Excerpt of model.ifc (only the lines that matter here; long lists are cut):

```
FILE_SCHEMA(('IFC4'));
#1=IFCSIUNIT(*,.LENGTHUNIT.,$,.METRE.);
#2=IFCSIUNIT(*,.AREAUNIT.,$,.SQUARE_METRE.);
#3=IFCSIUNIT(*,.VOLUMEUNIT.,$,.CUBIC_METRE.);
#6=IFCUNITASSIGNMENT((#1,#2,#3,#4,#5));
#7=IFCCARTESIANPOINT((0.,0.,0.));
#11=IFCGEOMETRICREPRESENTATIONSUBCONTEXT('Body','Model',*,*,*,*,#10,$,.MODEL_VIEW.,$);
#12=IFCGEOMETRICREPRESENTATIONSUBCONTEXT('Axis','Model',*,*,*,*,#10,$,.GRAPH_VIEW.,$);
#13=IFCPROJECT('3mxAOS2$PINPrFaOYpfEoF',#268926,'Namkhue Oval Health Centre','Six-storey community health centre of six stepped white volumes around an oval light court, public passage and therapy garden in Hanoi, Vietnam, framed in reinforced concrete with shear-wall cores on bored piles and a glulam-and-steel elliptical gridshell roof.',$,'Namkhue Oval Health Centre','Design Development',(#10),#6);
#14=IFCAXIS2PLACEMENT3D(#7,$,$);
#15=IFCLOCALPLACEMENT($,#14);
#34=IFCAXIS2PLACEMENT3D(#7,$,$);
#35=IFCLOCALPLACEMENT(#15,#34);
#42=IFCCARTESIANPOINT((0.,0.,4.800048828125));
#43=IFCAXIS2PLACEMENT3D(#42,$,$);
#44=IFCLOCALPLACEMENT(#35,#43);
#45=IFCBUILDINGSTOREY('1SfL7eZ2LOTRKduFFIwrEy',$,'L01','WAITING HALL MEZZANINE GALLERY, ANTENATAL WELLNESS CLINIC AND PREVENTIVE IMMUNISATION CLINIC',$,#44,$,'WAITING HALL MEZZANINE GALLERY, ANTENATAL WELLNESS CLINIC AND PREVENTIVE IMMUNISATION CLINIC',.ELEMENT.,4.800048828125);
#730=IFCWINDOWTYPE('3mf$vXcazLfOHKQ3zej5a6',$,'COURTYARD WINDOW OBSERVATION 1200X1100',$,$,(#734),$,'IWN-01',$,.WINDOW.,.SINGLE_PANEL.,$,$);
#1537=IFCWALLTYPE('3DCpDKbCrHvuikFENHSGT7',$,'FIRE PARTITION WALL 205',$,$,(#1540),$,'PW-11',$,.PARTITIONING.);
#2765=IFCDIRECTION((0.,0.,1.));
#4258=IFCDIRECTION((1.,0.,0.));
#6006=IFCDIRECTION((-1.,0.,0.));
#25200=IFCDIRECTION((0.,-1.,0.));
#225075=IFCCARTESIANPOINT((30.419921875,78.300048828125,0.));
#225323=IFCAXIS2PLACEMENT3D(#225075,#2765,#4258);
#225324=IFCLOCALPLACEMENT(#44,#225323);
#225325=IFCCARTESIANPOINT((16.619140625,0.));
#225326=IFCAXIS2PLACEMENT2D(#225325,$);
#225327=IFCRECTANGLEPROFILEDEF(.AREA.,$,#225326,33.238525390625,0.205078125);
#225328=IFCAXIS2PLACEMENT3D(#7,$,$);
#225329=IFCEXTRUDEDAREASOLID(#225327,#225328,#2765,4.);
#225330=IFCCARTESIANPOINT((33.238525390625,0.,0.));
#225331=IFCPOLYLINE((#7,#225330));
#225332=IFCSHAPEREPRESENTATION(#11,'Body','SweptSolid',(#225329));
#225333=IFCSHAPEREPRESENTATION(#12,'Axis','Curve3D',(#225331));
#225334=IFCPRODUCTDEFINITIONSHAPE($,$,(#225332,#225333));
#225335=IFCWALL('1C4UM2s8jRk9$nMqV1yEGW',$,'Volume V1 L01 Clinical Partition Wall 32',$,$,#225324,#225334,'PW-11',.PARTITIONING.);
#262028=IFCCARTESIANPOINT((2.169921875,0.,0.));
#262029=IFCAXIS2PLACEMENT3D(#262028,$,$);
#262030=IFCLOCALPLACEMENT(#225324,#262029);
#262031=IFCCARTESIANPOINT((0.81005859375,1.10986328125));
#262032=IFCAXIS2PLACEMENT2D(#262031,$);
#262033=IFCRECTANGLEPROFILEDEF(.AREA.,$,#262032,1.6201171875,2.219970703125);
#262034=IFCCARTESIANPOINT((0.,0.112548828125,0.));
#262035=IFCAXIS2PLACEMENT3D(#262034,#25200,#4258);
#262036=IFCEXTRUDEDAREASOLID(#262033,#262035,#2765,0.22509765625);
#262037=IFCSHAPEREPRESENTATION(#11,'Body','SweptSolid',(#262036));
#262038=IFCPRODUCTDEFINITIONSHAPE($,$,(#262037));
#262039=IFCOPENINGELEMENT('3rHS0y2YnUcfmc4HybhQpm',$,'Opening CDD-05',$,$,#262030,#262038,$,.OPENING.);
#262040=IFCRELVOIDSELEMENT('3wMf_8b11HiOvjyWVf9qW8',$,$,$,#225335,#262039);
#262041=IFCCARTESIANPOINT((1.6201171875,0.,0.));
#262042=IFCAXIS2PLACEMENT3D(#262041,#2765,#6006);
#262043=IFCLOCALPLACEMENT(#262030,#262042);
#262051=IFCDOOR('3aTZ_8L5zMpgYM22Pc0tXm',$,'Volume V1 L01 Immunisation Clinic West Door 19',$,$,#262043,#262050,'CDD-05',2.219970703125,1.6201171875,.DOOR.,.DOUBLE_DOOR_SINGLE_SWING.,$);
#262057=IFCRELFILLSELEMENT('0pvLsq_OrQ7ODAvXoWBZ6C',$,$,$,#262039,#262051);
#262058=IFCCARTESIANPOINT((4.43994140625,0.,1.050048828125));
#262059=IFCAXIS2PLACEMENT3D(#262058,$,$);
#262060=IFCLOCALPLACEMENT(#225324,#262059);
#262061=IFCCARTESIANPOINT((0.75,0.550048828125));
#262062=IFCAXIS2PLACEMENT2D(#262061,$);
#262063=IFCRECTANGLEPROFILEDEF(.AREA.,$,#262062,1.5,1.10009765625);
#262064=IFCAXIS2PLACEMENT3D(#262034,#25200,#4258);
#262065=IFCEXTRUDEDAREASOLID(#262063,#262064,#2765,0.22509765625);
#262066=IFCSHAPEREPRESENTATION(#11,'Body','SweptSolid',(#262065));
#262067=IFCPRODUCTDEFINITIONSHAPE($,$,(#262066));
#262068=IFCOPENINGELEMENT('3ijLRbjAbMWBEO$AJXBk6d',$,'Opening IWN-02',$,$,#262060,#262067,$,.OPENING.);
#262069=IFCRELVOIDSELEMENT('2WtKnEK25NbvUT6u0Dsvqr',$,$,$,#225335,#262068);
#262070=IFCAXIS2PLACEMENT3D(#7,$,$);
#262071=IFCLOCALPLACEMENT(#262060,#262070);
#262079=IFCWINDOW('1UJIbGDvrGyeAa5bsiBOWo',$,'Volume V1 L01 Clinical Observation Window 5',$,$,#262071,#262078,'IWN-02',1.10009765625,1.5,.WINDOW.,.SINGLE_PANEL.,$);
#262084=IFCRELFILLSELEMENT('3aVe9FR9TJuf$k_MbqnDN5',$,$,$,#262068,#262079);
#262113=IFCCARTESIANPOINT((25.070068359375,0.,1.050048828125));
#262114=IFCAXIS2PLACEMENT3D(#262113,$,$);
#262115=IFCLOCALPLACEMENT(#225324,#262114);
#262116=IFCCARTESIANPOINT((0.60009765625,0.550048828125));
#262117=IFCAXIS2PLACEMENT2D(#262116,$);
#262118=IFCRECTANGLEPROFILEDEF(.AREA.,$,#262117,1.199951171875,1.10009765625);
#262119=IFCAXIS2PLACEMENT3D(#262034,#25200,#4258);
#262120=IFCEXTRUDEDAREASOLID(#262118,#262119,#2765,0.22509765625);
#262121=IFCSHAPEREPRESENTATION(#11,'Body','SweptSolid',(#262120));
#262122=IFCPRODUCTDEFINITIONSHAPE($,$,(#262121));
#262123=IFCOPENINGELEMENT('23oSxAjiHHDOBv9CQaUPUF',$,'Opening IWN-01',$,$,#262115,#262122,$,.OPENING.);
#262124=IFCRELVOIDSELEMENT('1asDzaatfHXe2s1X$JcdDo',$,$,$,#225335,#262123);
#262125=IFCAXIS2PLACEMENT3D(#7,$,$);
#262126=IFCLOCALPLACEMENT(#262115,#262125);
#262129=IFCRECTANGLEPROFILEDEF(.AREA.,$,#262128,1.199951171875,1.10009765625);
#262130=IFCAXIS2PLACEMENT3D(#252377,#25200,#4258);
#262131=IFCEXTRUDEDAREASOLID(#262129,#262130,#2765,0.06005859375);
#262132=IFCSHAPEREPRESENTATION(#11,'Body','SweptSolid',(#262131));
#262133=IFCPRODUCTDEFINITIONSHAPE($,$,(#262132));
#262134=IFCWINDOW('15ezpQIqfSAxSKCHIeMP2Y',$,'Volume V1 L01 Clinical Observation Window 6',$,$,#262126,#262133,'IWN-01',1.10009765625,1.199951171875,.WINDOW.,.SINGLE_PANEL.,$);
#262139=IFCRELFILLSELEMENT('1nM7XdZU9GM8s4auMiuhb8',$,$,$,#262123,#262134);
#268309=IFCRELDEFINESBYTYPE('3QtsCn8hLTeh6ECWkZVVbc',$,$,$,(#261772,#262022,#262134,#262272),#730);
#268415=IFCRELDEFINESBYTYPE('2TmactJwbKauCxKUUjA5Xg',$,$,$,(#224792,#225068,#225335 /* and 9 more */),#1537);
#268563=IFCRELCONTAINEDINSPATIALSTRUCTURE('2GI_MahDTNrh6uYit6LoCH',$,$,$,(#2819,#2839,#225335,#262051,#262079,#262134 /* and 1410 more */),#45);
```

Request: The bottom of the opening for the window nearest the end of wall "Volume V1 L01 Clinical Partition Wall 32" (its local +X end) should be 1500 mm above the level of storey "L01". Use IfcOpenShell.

```python
import numpy as np
import ifcopenshell
import ifcopenshell.api.geometry
import ifcopenshell.geom
import ifcopenshell.util.element
import ifcopenshell.util.placement
import ifcopenshell.util.shape
import ifcopenshell.util.unit

model = ifcopenshell.open("model.ifc")
unit_scale = ifcopenshell.util.unit.calculate_unit_scale(model)

window = model.by_id(262134)
opening = window.FillsVoids[0].RelatingOpeningElement
storey = ifcopenshell.util.element.get_container(window, ifc_class="IfcBuildingStorey")
level = ifcopenshell.util.placement.get_local_placement(storey.ObjectPlacement)[2, 3]

# The opening's origin need not be at the sill, so measure its lowest point.
shape = ifcopenshell.geom.create_shape(ifcopenshell.geom.settings(), opening)
bottom = ifcopenshell.util.shape.get_shape_bottom_elevation(shape, shape.geometry) / unit_scale
dz = level + 1.5 - bottom

shift = np.array([0.0, 0.0, dz])
# The window is placed relative to its opening, so it follows when the opening moves.
matrix = ifcopenshell.util.placement.get_local_placement(opening.ObjectPlacement)
matrix[:3, 3] += shift
ifcopenshell.api.geometry.edit_object_placement(
    model, product=opening, matrix=matrix, is_si=False, should_transform_children=True
)

print(f"moved by {dz * unit_scale:+.3f} m")

model.write("model-out.ifc")
```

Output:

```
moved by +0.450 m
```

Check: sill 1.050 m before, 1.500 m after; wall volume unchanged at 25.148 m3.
